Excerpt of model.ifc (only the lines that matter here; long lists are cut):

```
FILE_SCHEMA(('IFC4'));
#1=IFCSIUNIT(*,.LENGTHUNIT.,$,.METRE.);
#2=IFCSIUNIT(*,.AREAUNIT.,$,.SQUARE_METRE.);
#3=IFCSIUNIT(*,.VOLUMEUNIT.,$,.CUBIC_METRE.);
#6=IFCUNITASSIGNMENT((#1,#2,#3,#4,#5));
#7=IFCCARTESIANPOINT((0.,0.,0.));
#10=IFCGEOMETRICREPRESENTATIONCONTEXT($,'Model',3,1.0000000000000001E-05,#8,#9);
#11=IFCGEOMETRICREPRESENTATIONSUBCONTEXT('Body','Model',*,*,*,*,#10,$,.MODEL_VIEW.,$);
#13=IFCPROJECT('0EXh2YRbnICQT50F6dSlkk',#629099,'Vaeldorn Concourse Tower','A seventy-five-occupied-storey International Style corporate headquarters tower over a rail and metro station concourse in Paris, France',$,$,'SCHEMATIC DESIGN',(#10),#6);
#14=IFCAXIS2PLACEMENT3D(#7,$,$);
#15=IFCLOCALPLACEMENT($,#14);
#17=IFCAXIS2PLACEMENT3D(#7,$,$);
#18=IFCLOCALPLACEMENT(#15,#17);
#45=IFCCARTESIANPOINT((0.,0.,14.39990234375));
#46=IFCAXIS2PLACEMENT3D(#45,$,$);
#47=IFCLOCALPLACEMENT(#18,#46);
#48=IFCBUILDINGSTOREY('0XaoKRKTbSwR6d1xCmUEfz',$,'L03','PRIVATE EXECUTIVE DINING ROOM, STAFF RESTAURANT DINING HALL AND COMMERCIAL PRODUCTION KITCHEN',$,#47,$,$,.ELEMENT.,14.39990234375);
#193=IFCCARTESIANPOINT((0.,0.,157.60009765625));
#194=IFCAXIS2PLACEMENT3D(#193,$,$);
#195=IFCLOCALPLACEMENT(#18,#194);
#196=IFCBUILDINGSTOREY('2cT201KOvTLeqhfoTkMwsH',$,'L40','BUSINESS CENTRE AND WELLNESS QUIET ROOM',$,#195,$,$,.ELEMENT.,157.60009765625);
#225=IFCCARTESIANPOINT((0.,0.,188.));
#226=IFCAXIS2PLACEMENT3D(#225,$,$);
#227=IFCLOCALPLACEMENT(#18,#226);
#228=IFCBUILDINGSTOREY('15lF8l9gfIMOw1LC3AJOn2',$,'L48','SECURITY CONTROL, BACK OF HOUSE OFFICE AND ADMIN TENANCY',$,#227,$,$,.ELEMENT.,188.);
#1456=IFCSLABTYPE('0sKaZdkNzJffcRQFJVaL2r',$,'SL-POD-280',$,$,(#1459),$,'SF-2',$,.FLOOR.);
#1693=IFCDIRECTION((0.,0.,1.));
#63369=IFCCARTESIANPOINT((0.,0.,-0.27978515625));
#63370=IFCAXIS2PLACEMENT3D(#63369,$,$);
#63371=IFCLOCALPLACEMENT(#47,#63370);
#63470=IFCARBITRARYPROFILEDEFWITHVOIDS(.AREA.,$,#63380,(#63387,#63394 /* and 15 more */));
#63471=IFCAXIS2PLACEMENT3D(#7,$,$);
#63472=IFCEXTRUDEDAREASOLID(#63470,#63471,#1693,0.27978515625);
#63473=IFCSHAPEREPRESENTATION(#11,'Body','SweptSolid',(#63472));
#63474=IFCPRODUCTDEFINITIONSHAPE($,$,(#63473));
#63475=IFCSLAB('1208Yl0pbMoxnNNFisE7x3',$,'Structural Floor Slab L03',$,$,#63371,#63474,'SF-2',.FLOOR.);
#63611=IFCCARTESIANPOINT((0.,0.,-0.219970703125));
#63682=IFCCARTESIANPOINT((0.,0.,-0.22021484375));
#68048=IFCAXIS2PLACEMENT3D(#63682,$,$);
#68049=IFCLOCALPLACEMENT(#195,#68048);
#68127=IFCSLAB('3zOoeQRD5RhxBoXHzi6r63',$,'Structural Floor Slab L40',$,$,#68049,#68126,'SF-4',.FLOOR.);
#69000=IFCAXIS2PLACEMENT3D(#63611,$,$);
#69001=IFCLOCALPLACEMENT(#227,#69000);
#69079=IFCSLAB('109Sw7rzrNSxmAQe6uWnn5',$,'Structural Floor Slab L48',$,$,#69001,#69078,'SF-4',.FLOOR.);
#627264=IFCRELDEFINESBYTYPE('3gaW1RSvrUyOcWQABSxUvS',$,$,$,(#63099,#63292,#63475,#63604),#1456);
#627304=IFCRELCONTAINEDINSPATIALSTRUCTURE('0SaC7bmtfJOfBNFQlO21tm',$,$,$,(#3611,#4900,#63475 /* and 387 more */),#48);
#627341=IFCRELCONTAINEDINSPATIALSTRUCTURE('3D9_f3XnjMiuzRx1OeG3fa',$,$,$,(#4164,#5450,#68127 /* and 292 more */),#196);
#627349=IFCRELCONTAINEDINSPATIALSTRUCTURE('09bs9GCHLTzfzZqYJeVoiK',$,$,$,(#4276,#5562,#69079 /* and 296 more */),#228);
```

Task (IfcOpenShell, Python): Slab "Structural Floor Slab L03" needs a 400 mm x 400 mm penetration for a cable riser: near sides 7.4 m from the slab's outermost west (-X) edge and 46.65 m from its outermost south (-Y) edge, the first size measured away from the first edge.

```python
import numpy as np
import ifcopenshell
import ifcopenshell.api.feature
import ifcopenshell.api.geometry
import ifcopenshell.api.root
import ifcopenshell.geom
import ifcopenshell.util.placement
import ifcopenshell.util.representation
import ifcopenshell.util.shape
import ifcopenshell.util.unit

model = ifcopenshell.open("model.ifc")
unit_scale = ifcopenshell.util.unit.calculate_unit_scale(model)
settings = ifcopenshell.geom.settings()


def volume(element):
    """Net volume in cubic metres, openings subtracted."""
    shape = ifcopenshell.geom.create_shape(settings, element)
    return ifcopenshell.util.shape.get_volume(shape.geometry)


slab = model.by_guid("1208Yl0pbMoxnNNFisE7x3")
before = volume(slab)

# Extent in the slab's own axes, in metres. The edges named are its -X and -Y sides.
slab_shape = ifcopenshell.geom.create_shape(settings, slab)
vertices = ifcopenshell.util.shape.get_vertices(slab_shape.geometry)
x_min, y_min, bottom = vertices.min(axis=0)
top = vertices[:, 2].max()

opening = ifcopenshell.api.root.create_entity(model, ifc_class="IfcOpeningElement", name="Cable riser opening", predefined_type="OPENING")
context = ifcopenshell.util.representation.get_context(model, "Model", "Body", "MODEL_VIEW")
width, depth = 0.4, 0.4
outline = [(0.0, 0.0), (width, 0.0), (width, depth), (0.0, depth), (0.0, 0.0)]
# Overshoot both faces by 50 mm so the cut is clean.
shape = ifcopenshell.api.geometry.add_slab_representation(
    model, context=context, depth=top - bottom + 0.1, polyline=outline
)
ifcopenshell.api.geometry.assign_representation(model, product=opening, representation=shape)

matrix = ifcopenshell.util.placement.get_local_placement(slab.ObjectPlacement)
matrix[:, 3] = matrix @ np.append(np.array([x_min + 7.4, y_min + 46.65, bottom - 0.05]) / unit_scale, 1.0)
ifcopenshell.api.geometry.edit_object_placement(model, product=opening, matrix=matrix, is_si=False)
ifcopenshell.api.feature.add_feature(model, feature=opening, element=slab)

after = volume(slab)

print(f"slab volume {before:.3f} -> {after:.3f} m3")

model.write("model_edited.ifc")
```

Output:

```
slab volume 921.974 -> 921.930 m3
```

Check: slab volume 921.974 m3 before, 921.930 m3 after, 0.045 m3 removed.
